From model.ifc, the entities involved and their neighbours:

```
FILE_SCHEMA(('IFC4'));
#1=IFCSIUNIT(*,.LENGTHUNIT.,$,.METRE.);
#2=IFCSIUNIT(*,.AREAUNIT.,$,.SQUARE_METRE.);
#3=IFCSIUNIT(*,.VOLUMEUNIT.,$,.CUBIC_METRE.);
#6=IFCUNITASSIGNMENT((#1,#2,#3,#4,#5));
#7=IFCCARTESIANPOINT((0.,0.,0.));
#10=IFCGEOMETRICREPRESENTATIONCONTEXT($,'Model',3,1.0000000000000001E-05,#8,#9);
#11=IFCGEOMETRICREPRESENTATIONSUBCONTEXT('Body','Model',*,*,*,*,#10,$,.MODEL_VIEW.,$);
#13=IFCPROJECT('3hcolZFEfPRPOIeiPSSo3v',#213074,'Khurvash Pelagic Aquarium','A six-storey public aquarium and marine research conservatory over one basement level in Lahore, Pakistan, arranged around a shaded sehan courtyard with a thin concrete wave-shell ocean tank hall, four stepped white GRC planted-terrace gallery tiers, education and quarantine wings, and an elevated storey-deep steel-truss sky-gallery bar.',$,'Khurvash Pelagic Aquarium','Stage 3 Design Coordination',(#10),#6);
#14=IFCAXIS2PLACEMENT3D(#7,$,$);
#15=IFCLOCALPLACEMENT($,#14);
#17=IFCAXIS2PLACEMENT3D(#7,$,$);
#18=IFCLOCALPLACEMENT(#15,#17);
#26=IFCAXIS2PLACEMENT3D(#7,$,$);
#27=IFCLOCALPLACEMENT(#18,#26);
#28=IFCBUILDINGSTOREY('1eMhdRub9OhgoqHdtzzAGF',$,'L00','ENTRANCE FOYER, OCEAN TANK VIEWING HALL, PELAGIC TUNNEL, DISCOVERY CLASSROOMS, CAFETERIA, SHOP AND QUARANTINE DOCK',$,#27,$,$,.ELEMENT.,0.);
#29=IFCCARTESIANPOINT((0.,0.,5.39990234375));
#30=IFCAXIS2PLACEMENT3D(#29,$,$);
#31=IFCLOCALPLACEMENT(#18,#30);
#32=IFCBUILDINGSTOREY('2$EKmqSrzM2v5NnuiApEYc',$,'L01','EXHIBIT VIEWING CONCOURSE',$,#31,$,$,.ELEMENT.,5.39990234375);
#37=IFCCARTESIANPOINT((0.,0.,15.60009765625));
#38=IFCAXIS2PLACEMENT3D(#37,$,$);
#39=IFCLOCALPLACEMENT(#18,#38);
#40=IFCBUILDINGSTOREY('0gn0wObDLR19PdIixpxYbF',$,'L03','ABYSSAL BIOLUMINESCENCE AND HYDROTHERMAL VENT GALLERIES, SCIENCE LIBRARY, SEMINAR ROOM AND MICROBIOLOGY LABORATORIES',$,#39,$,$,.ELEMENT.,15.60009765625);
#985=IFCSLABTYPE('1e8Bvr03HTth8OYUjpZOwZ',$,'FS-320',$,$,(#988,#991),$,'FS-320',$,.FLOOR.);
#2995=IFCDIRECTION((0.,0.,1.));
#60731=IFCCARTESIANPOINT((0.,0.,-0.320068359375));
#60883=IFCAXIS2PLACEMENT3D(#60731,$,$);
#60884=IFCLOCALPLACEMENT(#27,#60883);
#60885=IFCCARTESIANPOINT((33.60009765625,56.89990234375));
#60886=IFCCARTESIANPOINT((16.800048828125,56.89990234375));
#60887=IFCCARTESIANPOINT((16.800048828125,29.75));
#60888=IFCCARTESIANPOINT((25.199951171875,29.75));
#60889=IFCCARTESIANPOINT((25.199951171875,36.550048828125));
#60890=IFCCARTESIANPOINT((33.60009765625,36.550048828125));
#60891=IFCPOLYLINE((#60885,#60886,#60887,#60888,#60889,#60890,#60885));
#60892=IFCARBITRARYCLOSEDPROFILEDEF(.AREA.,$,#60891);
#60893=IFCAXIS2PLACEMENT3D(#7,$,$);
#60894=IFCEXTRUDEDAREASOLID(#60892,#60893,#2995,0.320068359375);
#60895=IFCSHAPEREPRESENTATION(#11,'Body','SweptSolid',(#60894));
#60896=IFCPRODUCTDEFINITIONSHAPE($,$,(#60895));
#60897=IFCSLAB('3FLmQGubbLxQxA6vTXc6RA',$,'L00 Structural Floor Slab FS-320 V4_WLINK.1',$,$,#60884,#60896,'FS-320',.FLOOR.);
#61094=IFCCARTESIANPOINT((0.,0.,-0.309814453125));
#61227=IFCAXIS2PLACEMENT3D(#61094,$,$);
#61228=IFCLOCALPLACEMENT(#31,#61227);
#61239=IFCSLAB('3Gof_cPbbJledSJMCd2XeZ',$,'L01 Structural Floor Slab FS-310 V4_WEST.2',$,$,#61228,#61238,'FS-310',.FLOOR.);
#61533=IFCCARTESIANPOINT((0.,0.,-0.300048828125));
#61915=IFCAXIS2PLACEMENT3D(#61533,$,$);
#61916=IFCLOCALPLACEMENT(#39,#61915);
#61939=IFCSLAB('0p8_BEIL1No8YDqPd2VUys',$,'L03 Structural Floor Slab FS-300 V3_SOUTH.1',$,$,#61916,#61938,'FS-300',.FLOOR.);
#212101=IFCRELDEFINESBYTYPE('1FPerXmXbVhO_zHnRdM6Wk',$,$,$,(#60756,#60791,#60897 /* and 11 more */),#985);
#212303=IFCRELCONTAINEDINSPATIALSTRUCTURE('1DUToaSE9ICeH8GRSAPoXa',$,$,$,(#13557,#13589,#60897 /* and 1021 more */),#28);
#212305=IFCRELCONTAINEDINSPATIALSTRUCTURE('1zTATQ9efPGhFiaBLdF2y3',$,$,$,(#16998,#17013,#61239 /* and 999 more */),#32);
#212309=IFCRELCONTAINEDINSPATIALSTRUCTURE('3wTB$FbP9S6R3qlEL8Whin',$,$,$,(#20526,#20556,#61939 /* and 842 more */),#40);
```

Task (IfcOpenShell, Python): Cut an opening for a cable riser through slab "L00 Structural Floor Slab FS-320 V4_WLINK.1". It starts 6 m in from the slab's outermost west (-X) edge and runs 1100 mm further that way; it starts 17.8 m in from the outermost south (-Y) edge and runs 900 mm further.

```python
import numpy as np
import ifcopenshell
import ifcopenshell.api.feature
import ifcopenshell.api.geometry
import ifcopenshell.api.root
import ifcopenshell.geom
import ifcopenshell.util.placement
import ifcopenshell.util.representation
import ifcopenshell.util.shape
import ifcopenshell.util.unit

model = ifcopenshell.open("model.ifc")
unit_scale = ifcopenshell.util.unit.calculate_unit_scale(model)
settings = ifcopenshell.geom.settings()


def volume(element):
    """Net volume in cubic metres, openings subtracted."""
    shape = ifcopenshell.geom.create_shape(settings, element)
    return ifcopenshell.util.shape.get_volume(shape.geometry)


slab = model.by_guid("3FLmQGubbLxQxA6vTXc6RA")
before = volume(slab)

# Extent in the slab's own axes, in metres. The edges named are its -X and -Y sides.
slab_shape = ifcopenshell.geom.create_shape(settings, slab)
vertices = ifcopenshell.util.shape.get_vertices(slab_shape.geometry)
x_min, y_min, bottom = vertices.min(axis=0)
top = vertices[:, 2].max()

opening = ifcopenshell.api.root.create_entity(model, ifc_class="IfcOpeningElement", name="Cable riser opening", predefined_type="OPENING")
context = ifcopenshell.util.representation.get_context(model, "Model", "Body", "MODEL_VIEW")
width, depth = 1.1, 0.9
outline = [(0.0, 0.0), (width, 0.0), (width, depth), (0.0, depth), (0.0, 0.0)]
# Overshoot both faces by 50 mm so the cut is clean.
shape = ifcopenshell.api.geometry.add_slab_representation(
    model, context=context, depth=top - bottom + 0.1, polyline=outline
)
ifcopenshell.api.geometry.assign_representation(model, product=opening, representation=shape)

matrix = ifcopenshell.util.placement.get_local_placement(slab.ObjectPlacement)
matrix[:, 3] = matrix @ np.append(np.array([x_min + 6, y_min + 17.8, bottom - 0.05]) / unit_scale, 1.0)
ifcopenshell.api.geometry.edit_object_placement(model, product=opening, matrix=matrix, is_si=False)
ifcopenshell.api.feature.add_feature(model, feature=opening, element=slab)

after = volume(slab)

print(f"slab volume {before:.3f} -> {after:.3f} m3")

model.write("model_updated.ifc")
```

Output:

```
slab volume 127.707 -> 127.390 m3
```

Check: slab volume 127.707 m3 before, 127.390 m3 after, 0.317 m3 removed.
